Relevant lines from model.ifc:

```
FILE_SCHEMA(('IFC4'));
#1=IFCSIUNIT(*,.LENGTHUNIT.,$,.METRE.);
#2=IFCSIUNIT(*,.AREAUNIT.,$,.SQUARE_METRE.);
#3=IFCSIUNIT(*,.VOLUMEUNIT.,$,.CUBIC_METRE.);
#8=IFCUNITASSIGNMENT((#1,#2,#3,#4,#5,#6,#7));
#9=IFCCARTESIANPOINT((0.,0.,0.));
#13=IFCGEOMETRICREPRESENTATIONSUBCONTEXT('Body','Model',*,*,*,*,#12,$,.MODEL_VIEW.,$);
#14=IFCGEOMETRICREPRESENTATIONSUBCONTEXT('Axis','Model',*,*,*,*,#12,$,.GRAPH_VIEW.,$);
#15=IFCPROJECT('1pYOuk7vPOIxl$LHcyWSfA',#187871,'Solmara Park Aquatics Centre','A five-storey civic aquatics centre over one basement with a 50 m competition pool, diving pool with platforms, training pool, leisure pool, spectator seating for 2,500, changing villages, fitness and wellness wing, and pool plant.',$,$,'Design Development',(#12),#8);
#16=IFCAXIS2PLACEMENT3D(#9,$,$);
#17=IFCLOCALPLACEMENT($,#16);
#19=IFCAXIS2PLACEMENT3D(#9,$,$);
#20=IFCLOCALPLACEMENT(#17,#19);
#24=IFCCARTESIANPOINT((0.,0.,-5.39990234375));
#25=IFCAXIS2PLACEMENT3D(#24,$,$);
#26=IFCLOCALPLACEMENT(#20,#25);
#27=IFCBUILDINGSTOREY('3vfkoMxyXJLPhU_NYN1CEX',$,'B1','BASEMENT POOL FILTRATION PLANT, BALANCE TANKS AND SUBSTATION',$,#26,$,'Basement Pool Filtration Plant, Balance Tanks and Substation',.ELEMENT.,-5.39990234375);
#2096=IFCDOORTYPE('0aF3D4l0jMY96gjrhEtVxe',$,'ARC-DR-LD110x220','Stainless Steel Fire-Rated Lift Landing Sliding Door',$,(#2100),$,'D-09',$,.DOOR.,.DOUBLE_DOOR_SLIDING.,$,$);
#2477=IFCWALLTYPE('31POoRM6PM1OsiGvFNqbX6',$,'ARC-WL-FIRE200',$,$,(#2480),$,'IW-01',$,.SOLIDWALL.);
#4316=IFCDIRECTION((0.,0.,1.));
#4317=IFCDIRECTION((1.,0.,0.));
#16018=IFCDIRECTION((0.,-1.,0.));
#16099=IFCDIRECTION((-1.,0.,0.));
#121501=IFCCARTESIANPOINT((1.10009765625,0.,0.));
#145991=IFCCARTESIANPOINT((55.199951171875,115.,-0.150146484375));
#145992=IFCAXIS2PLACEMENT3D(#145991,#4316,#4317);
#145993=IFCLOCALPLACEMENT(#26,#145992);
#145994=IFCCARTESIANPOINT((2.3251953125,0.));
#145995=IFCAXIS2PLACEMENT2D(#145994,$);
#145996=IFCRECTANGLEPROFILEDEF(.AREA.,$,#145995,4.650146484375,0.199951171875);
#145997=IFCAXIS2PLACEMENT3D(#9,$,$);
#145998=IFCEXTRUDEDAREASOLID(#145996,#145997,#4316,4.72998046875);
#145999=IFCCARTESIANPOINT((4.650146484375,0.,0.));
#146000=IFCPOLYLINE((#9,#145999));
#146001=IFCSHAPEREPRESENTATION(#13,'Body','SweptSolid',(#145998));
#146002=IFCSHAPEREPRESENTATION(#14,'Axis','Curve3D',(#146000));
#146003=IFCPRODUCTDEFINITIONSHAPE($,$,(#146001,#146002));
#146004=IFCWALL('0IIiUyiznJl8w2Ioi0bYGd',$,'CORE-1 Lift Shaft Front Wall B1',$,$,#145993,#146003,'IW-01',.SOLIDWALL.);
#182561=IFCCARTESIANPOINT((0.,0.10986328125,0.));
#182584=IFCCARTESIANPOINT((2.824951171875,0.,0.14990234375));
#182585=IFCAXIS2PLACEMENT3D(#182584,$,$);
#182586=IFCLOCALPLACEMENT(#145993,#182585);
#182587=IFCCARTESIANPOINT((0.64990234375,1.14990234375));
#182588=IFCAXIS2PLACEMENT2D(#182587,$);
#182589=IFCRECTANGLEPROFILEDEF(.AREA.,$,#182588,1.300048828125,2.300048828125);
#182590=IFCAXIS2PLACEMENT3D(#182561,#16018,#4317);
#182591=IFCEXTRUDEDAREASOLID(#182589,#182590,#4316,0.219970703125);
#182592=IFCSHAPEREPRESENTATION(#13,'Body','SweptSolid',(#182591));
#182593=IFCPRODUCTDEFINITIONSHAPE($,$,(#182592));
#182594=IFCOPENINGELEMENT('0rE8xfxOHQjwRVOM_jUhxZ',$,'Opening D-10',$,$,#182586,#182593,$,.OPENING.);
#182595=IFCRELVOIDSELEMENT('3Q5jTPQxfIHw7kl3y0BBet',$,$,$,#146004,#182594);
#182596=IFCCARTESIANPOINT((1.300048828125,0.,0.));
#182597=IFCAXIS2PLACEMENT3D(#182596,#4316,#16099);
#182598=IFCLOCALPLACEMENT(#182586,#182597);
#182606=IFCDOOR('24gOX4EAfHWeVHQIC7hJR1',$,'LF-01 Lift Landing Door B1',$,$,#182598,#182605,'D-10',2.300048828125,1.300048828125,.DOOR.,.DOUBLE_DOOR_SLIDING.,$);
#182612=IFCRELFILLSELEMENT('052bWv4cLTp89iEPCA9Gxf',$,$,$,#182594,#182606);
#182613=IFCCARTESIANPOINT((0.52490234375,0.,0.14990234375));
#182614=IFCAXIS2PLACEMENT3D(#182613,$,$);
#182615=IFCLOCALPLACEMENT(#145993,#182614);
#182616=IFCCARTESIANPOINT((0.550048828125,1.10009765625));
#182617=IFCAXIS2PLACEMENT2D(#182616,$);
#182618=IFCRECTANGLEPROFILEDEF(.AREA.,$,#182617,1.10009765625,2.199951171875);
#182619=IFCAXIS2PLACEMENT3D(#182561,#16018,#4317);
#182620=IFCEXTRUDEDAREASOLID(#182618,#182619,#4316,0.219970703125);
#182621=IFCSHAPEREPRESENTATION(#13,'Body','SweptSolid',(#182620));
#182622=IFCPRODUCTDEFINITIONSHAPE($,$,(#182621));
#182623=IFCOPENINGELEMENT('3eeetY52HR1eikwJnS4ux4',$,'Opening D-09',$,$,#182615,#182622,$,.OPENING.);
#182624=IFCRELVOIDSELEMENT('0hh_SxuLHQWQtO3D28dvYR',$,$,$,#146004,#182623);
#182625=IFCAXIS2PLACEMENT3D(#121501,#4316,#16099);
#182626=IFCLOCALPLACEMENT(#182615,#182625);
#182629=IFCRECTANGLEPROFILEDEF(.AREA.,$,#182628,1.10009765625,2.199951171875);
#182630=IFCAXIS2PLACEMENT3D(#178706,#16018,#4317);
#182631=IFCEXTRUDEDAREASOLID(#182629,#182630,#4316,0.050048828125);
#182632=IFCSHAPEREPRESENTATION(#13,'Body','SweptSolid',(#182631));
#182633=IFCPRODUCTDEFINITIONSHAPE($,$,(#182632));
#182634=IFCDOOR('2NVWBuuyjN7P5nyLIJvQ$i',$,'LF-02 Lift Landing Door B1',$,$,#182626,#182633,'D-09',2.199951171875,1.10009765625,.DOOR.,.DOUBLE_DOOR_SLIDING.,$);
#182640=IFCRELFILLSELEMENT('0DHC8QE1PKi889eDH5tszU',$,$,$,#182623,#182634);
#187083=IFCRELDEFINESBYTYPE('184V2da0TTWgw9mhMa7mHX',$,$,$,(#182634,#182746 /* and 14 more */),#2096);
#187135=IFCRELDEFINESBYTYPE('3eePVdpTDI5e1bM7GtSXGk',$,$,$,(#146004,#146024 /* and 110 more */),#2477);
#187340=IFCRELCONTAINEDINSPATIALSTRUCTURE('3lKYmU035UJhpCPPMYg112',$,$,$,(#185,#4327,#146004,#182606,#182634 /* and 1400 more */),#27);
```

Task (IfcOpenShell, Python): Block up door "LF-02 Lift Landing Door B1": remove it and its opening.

```python
import ifcopenshell
import ifcopenshell.api.feature
import ifcopenshell.api.root
import ifcopenshell.geom
import ifcopenshell.util.shape

model = ifcopenshell.open("model.ifc")
settings = ifcopenshell.geom.settings()


def volume(element):
    """Net volume in cubic metres, openings subtracted."""
    shape = ifcopenshell.geom.create_shape(settings, element)
    return ifcopenshell.util.shape.get_volume(shape.geometry)


door = model.by_guid("2NVWBuuyjN7P5nyLIJvQ$i")
opening = door.FillsVoids[0].RelatingOpeningElement
wall = opening.VoidsElements[0].RelatingBuildingElement
before = volume(wall)

ifcopenshell.api.root.remove_product(model, product=door)
ifcopenshell.api.feature.remove_feature(model, feature=opening)

after = volume(wall)

print(f"wall volume {before:.3f} -> {after:.3f} m3")

model.write("model_updated.ifc")
```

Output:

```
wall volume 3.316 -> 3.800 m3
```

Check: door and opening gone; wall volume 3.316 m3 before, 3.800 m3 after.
